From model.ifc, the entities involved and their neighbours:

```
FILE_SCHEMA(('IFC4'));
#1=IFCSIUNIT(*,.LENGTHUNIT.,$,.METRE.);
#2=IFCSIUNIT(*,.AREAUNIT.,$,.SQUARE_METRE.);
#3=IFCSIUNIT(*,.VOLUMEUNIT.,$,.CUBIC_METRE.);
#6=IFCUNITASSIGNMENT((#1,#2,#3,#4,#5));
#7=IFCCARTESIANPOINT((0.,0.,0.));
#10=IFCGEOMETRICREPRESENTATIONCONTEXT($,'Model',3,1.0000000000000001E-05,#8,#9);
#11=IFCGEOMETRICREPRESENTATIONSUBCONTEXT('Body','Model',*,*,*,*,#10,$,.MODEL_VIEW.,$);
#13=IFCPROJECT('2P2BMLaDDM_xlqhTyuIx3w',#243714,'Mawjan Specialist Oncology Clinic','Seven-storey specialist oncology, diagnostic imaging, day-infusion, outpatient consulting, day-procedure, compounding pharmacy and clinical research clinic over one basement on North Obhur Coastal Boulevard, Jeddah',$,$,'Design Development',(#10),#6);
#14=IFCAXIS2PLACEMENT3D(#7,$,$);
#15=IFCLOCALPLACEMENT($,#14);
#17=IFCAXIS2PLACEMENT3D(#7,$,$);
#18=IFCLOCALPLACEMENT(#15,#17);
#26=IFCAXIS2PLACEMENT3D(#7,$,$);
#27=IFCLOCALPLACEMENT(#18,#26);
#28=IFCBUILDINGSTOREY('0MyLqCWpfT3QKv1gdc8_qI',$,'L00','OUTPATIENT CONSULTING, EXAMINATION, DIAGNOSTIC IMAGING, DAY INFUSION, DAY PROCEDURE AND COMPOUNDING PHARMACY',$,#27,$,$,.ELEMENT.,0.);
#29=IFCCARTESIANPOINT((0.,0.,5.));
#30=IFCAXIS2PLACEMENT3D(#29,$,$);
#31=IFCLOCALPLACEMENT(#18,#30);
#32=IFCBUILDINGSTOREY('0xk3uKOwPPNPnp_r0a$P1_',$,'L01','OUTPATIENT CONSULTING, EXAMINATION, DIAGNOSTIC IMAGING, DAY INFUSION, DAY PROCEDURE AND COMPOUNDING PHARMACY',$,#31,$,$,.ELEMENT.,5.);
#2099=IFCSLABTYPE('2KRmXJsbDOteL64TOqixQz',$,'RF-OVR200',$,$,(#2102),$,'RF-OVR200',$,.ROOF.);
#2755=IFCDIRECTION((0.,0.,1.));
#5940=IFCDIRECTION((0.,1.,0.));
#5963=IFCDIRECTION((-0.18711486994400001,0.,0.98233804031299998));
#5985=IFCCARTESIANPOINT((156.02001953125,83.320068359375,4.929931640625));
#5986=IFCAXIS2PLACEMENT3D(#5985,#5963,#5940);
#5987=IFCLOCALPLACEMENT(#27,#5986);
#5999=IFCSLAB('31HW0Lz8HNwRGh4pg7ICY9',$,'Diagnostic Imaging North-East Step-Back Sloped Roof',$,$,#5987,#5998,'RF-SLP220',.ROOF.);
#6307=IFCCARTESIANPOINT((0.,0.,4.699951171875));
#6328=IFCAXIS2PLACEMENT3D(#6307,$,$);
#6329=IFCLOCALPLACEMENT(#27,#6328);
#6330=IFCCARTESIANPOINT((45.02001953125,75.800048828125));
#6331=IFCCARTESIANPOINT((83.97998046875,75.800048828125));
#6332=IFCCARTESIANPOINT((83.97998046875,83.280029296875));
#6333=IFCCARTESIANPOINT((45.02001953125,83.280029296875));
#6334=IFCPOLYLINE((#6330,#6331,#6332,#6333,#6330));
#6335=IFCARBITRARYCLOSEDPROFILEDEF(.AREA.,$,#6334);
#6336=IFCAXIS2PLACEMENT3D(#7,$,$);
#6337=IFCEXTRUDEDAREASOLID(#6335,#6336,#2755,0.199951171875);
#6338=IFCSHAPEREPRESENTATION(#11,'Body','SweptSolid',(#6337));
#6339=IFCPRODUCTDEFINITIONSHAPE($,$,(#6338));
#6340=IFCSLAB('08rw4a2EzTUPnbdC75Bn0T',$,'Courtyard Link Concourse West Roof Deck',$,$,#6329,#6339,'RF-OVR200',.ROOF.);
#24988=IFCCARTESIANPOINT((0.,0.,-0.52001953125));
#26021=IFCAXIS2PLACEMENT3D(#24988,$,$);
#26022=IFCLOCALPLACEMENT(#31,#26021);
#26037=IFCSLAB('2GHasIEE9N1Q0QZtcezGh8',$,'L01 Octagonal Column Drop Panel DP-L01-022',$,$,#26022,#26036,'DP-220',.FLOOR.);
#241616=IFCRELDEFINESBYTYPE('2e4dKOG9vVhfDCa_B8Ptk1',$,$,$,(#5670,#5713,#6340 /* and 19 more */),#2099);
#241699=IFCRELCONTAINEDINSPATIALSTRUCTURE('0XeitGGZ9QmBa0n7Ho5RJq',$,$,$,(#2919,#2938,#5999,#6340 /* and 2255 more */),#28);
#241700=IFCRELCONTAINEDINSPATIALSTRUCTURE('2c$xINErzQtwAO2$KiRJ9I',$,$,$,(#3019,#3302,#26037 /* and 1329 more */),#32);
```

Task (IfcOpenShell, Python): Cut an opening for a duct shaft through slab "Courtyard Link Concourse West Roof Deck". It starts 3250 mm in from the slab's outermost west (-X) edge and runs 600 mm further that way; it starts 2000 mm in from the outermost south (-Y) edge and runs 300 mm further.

```python
import numpy as np
import ifcopenshell
import ifcopenshell.api.feature
import ifcopenshell.api.geometry
import ifcopenshell.api.root
import ifcopenshell.geom
import ifcopenshell.util.placement
import ifcopenshell.util.representation
import ifcopenshell.util.shape
import ifcopenshell.util.unit

model = ifcopenshell.open("model.ifc")
unit_scale = ifcopenshell.util.unit.calculate_unit_scale(model)
settings = ifcopenshell.geom.settings()


def volume(element):
    """Net volume in cubic metres, openings subtracted."""
    shape = ifcopenshell.geom.create_shape(settings, element)
    return ifcopenshell.util.shape.get_volume(shape.geometry)


slab = model.by_guid("08rw4a2EzTUPnbdC75Bn0T")
before = volume(slab)

# Extent in the slab's own axes, in metres. The edges named are its -X and -Y sides.
slab_shape = ifcopenshell.geom.create_shape(settings, slab)
vertices = ifcopenshell.util.shape.get_vertices(slab_shape.geometry)
x_min, y_min, bottom = vertices.min(axis=0)
top = vertices[:, 2].max()

opening = ifcopenshell.api.root.create_entity(model, ifc_class="IfcOpeningElement", name="Duct shaft opening", predefined_type="OPENING")
context = ifcopenshell.util.representation.get_context(model, "Model", "Body", "MODEL_VIEW")
width, depth = 0.6, 0.3
outline = [(0.0, 0.0), (width, 0.0), (width, depth), (0.0, depth), (0.0, 0.0)]
# Overshoot both faces by 50 mm so the cut is clean.
shape = ifcopenshell.api.geometry.add_slab_representation(
    model, context=context, depth=top - bottom + 0.1, polyline=outline
)
ifcopenshell.api.geometry.assign_representation(model, product=opening, representation=shape)

matrix = ifcopenshell.util.placement.get_local_placement(slab.ObjectPlacement)
matrix[:, 3] = matrix @ np.append(np.array([x_min + 3.25, y_min + 2, bottom - 0.05]) / unit_scale, 1.0)
ifcopenshell.api.geometry.edit_object_placement(model, product=opening, matrix=matrix, is_si=False)
ifcopenshell.api.feature.add_feature(model, feature=opening, element=slab)

after = volume(slab)

print(f"slab volume {before:.3f} -> {after:.3f} m3")

model.write("model_updated.ifc")
```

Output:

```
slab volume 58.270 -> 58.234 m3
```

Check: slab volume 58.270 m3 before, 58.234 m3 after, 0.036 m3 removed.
